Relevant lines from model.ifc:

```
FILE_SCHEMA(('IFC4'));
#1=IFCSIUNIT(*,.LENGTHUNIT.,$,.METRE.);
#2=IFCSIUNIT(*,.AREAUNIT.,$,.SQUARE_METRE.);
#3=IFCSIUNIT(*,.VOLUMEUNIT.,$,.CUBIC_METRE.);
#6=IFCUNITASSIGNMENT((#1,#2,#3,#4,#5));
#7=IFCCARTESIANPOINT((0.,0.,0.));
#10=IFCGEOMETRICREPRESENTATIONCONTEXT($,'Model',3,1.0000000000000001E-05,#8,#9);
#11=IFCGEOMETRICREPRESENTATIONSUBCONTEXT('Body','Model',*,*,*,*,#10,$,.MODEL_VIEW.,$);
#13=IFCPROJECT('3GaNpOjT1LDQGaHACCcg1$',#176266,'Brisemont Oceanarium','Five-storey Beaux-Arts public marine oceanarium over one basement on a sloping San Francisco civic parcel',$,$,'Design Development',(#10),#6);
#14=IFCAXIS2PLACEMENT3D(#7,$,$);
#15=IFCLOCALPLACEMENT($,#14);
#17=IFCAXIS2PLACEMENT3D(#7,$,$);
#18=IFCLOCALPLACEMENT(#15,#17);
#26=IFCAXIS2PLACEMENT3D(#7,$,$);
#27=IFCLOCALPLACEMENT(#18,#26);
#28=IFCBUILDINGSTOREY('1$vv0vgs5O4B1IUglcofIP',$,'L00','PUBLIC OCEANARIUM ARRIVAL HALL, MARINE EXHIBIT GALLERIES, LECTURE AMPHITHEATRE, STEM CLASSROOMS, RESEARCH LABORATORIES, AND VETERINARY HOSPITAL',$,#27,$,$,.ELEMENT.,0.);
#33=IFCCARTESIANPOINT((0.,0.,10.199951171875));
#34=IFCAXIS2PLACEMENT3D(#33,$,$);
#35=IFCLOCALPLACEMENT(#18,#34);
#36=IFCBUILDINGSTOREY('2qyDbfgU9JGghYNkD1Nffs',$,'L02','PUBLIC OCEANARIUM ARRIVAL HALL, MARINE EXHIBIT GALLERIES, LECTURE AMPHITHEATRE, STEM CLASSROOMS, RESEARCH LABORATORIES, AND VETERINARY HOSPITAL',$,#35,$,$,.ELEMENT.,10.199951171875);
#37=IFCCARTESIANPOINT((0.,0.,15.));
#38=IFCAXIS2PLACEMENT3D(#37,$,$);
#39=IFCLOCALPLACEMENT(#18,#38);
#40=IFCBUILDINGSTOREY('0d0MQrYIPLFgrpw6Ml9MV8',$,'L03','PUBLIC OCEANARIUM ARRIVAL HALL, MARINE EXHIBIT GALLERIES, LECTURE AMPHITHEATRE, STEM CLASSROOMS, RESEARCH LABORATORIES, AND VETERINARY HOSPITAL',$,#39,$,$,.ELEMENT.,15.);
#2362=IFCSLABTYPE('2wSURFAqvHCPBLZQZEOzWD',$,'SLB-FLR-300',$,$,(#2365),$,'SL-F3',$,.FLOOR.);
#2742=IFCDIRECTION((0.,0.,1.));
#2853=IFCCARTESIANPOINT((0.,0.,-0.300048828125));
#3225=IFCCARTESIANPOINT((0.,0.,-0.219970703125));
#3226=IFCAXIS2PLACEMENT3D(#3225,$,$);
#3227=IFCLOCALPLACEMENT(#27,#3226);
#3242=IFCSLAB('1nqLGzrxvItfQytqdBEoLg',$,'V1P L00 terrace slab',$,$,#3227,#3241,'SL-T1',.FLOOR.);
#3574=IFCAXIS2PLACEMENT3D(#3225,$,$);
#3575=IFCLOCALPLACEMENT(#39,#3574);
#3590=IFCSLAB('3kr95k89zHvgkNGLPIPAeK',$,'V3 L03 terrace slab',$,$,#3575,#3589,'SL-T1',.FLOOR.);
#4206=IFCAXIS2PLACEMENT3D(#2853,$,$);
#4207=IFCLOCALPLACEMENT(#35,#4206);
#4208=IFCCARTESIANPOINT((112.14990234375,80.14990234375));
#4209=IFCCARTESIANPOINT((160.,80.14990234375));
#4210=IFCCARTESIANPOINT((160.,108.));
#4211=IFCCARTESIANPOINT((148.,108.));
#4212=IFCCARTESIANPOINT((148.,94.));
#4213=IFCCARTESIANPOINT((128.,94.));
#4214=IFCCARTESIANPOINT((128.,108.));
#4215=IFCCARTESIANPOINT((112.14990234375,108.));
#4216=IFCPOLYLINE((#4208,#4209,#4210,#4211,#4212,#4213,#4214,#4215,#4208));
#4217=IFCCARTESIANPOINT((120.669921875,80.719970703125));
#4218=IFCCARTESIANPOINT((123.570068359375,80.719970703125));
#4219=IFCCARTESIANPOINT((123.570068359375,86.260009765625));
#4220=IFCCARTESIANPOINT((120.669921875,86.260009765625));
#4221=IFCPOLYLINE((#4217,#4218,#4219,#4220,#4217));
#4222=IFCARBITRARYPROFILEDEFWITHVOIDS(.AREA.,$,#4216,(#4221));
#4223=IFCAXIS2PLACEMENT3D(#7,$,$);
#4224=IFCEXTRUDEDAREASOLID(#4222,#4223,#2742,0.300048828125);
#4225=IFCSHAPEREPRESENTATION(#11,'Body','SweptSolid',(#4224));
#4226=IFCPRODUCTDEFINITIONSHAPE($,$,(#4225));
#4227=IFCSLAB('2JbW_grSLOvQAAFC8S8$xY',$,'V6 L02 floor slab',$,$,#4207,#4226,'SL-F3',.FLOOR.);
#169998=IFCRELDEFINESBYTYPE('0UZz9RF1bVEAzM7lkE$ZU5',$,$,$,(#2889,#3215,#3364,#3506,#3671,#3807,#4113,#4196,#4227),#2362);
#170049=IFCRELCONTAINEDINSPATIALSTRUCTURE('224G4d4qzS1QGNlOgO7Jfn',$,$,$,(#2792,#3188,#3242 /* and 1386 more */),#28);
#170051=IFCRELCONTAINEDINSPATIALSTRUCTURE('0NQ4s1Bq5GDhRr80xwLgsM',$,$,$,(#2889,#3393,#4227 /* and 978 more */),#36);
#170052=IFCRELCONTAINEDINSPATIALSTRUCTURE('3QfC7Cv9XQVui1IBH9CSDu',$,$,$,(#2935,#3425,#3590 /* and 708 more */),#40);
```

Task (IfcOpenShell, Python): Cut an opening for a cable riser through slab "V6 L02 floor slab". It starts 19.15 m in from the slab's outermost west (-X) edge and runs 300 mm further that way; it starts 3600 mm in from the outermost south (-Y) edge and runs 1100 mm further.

```python
import numpy as np
import ifcopenshell
import ifcopenshell.api.feature
import ifcopenshell.api.geometry
import ifcopenshell.api.root
import ifcopenshell.geom
import ifcopenshell.util.placement
import ifcopenshell.util.representation
import ifcopenshell.util.shape
import ifcopenshell.util.unit

model = ifcopenshell.open("model.ifc")
unit_scale = ifcopenshell.util.unit.calculate_unit_scale(model)
settings = ifcopenshell.geom.settings()


def volume(element):
    """Net volume in cubic metres, openings subtracted."""
    shape = ifcopenshell.geom.create_shape(settings, element)
    return ifcopenshell.util.shape.get_volume(shape.geometry)


slab = model.by_guid("2JbW_grSLOvQAAFC8S8$xY")
before = volume(slab)

# Extent in the slab's own axes, in metres. The edges named are its -X and -Y sides.
slab_shape = ifcopenshell.geom.create_shape(settings, slab)
vertices = ifcopenshell.util.shape.get_vertices(slab_shape.geometry)
x_min, y_min, bottom = vertices.min(axis=0)
top = vertices[:, 2].max()

opening = ifcopenshell.api.root.create_entity(model, ifc_class="IfcOpeningElement", name="Cable riser opening", predefined_type="OPENING")
context = ifcopenshell.util.representation.get_context(model, "Model", "Body", "MODEL_VIEW")
width, depth = 0.3, 1.1
outline = [(0.0, 0.0), (width, 0.0), (width, depth), (0.0, depth), (0.0, 0.0)]
# Overshoot both faces by 50 mm so the cut is clean.
shape = ifcopenshell.api.geometry.add_slab_representation(
    model, context=context, depth=top - bottom + 0.1, polyline=outline
)
ifcopenshell.api.geometry.assign_representation(model, product=opening, representation=shape)

matrix = ifcopenshell.util.placement.get_local_placement(slab.ObjectPlacement)
matrix[:, 3] = matrix @ np.append(np.array([x_min + 19.15, y_min + 3.6, bottom - 0.05]) / unit_scale, 1.0)
ifcopenshell.api.geometry.edit_object_placement(model, product=opening, matrix=matrix, is_si=False)
ifcopenshell.api.feature.add_feature(model, feature=opening, element=slab)

after = volume(slab)

print(f"slab volume {before:.3f} -> {after:.3f} m3")

model.write("model_updated.ifc")
```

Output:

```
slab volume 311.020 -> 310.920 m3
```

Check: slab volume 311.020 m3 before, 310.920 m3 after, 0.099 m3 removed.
